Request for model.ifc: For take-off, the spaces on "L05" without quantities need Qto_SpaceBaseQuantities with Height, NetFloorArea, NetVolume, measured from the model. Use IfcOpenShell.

First a look at what the model holds.

```python
import ifcopenshell
import ifcopenshell.util.element
import ifcopenshell.util.unit

model = ifcopenshell.open("model.ifc")
print(model.schema)
for unit_type in ("LENGTHUNIT", "AREAUNIT", "VOLUMEUNIT"):
    print(unit_type, ifcopenshell.util.unit.calculate_unit_scale(model, unit_type))
storey = next(s for s in model.by_type("IfcBuildingStorey") if s.Name == "L05")
spaces = [e for e in ifcopenshell.util.element.get_decomposition(storey) if e.is_a("IfcSpace")]
for e in sorted(spaces, key=lambda e: e.id()):
    print(e.id(), e.is_a(), e.Name, list(ifcopenshell.util.element.get_psets(e, qtos_only=True)), sep=" | ")
```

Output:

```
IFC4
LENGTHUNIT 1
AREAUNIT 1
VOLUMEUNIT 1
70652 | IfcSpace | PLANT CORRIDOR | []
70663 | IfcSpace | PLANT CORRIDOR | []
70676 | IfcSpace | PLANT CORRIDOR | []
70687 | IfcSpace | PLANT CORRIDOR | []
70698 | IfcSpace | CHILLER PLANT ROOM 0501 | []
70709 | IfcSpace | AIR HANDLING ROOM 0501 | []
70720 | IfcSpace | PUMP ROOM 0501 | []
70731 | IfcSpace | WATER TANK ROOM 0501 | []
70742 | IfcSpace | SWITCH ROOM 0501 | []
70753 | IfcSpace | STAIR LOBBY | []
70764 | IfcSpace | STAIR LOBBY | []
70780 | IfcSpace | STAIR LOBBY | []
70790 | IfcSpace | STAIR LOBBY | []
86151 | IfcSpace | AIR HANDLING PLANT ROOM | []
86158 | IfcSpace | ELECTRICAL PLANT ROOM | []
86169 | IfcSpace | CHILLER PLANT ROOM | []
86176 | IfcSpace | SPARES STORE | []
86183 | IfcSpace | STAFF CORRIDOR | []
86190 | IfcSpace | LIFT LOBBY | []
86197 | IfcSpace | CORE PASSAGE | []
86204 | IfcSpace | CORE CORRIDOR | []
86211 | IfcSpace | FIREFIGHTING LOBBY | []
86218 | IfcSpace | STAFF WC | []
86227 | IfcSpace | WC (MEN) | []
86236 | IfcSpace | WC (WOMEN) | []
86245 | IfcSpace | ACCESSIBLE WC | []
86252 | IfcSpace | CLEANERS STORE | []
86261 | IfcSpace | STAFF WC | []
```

```python
import ifcopenshell
import ifcopenshell.api.pset
import ifcopenshell.geom
import ifcopenshell.util.element
import ifcopenshell.util.shape
import ifcopenshell.util.unit

model = ifcopenshell.open("model.ifc")
unit_scale = ifcopenshell.util.unit.calculate_unit_scale(model)
area_scale = ifcopenshell.util.unit.calculate_unit_scale(model, "AREAUNIT")
volume_scale = ifcopenshell.util.unit.calculate_unit_scale(model, "VOLUMEUNIT")
settings = ifcopenshell.geom.settings()

storey = next(s for s in model.by_type("IfcBuildingStorey") if s.Name == "L05")
spaces = [e for e in ifcopenshell.util.element.get_decomposition(storey) if e.is_a("IfcSpace")]

for e in sorted(spaces, key=lambda e: e.id()):
    if ifcopenshell.util.element.get_psets(e, qtos_only=True, should_inherit=False):
        continue
    # Geometry comes back in metres, in the element's own axes.
    shape = ifcopenshell.geom.create_shape(settings, e)
    values = {
        "Height": ifcopenshell.util.shape.get_z(shape.geometry) / unit_scale,
        "NetFloorArea": ifcopenshell.util.shape.get_footprint_area(shape.geometry) / area_scale,
        "NetVolume": ifcopenshell.util.shape.get_volume(shape.geometry) / volume_scale,
    }
    qto = ifcopenshell.api.pset.add_qto(model, product=e, name="Qto_SpaceBaseQuantities")
    ifcopenshell.api.pset.edit_qto(model, qto=qto, properties=values)
    print(e.id(), {k: round(v, 3) for k, v in values.items()})

model.write("model_edited.ifc")
```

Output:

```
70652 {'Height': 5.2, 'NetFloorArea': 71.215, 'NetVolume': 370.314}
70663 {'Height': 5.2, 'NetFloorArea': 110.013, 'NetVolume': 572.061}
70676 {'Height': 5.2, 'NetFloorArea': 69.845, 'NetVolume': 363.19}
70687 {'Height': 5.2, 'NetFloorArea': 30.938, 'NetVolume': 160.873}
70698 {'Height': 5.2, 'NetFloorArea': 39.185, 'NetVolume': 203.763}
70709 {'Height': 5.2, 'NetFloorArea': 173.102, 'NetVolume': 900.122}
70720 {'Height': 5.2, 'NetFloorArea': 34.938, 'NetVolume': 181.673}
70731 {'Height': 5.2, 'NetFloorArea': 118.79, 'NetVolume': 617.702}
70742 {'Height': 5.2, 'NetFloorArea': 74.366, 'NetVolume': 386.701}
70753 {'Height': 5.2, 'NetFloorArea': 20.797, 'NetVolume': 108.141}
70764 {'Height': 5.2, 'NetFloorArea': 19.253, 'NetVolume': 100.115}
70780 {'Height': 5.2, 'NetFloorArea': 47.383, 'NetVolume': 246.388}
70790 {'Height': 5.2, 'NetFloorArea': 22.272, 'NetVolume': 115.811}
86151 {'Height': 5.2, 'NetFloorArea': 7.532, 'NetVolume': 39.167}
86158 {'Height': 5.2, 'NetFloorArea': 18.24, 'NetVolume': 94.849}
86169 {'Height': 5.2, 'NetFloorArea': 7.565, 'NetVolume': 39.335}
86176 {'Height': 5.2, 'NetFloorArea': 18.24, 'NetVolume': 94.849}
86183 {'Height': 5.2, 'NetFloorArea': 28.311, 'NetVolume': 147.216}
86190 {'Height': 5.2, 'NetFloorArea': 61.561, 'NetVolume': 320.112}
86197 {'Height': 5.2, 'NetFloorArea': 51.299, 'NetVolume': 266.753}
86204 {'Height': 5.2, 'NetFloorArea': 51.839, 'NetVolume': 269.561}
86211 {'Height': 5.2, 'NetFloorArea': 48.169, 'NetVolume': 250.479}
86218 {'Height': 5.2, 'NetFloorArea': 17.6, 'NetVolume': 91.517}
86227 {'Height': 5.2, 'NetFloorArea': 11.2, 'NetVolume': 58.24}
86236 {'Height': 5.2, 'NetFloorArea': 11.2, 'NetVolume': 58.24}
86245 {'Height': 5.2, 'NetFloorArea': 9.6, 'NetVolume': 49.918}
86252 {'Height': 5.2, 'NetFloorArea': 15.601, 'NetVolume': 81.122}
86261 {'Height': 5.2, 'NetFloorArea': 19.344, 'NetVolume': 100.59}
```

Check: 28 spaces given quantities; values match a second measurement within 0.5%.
